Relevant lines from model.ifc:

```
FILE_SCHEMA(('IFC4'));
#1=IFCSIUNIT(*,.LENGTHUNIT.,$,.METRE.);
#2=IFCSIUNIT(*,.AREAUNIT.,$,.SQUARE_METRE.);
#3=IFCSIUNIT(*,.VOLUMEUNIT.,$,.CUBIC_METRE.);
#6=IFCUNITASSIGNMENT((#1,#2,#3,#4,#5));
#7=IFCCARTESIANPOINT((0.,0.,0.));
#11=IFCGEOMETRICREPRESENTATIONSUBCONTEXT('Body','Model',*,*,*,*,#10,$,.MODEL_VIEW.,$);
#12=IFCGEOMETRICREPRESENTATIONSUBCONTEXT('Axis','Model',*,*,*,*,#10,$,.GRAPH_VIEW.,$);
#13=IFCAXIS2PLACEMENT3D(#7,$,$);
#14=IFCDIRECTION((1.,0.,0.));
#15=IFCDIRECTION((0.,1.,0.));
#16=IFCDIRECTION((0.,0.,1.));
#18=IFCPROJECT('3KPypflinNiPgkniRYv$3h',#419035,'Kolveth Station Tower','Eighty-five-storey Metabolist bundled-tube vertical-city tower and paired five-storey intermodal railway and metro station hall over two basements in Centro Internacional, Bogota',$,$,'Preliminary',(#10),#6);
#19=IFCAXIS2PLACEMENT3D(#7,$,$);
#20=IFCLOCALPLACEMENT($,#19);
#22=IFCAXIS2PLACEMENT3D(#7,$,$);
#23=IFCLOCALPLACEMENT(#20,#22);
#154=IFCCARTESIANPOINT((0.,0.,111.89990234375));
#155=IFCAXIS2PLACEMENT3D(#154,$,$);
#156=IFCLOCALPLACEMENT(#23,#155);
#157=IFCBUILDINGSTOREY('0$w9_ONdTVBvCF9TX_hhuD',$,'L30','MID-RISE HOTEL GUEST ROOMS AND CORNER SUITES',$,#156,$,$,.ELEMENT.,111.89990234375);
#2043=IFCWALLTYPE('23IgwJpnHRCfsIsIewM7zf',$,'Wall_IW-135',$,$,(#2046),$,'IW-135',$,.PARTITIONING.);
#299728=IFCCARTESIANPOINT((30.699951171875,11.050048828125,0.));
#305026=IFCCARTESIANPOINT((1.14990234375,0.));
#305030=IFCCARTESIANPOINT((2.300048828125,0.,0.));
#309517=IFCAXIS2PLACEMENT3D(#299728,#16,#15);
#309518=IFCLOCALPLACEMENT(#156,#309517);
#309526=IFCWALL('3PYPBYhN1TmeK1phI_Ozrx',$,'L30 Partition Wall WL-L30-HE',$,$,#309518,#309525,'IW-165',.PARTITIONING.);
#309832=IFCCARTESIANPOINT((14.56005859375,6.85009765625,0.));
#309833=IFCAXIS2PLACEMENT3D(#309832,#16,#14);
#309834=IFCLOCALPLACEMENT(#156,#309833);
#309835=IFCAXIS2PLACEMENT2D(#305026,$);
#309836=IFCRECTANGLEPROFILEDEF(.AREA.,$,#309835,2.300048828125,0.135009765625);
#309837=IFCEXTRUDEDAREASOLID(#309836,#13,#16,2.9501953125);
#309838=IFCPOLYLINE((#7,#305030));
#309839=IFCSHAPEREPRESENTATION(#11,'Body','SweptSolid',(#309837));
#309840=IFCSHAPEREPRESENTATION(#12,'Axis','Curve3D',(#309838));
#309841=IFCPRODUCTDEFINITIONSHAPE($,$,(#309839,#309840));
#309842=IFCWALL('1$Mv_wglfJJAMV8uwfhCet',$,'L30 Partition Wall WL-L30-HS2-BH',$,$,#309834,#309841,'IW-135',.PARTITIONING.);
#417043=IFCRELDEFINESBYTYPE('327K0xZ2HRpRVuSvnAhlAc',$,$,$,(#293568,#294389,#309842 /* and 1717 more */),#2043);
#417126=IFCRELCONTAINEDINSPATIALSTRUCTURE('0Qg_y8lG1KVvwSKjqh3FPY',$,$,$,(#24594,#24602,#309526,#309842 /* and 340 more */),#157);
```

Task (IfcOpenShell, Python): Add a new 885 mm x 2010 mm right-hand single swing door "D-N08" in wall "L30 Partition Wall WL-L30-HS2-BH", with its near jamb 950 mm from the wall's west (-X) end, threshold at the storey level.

```python
import numpy as np
import ifcopenshell
import ifcopenshell.api.feature
import ifcopenshell.api.geometry
import ifcopenshell.api.root
import ifcopenshell.api.spatial
import ifcopenshell.geom
import ifcopenshell.util.element
import ifcopenshell.util.placement
import ifcopenshell.util.representation
import ifcopenshell.util.shape
import ifcopenshell.util.unit

model = ifcopenshell.open("model.ifc")
unit_scale = ifcopenshell.util.unit.calculate_unit_scale(model)
settings = ifcopenshell.geom.settings()


def volume(element):
    """Net volume in cubic metres, openings subtracted."""
    shape = ifcopenshell.geom.create_shape(settings, element)
    return ifcopenshell.util.shape.get_volume(shape.geometry)


wall = model.by_guid("1$Mv_wglfJJAMV8uwfhCet")
storey = ifcopenshell.util.element.get_container(wall, ifc_class="IfcBuildingStorey")
context = ifcopenshell.util.representation.get_context(model, "Model", "Body", "MODEL_VIEW")
before = volume(wall)

width, height, from_end, sill = 0.885, 2.01, 0.95, 0.0  # metres

# The wall runs along its own X axis, and the end named is its -X end.
wall_shape = ifcopenshell.geom.create_shape(settings, wall)
x, y, z = ifcopenshell.util.shape.get_vertices(wall_shape.geometry).T
start = x.min() + from_end
face, thickness = float(y.min()), float(y.max() - y.min())
wall_matrix = ifcopenshell.util.placement.get_local_placement(wall.ObjectPlacement)
level = ifcopenshell.util.placement.get_local_placement(storey.ObjectPlacement)[2, 3]


def in_wall(x, y):
    """Placement at x, y metres in the wall's axes, at sill height."""
    matrix = wall_matrix.copy()
    matrix[:, 3] = wall_matrix @ np.array([x / unit_scale, y / unit_scale, 0.0, 1.0])
    matrix[2, 3] = level + sill / unit_scale
    return matrix


# Opening: a box that overshoots both wall faces by 50 mm.
opening = ifcopenshell.api.root.create_entity(model, ifc_class="IfcOpeningElement", predefined_type="OPENING")
box = ifcopenshell.api.geometry.add_wall_representation(
    model, context=context, length=width, height=height, thickness=thickness + 0.1
)
ifcopenshell.api.geometry.assign_representation(model, product=opening, representation=box)
ifcopenshell.api.geometry.edit_object_placement(model, product=opening, matrix=in_wall(start, face - 0.05), is_si=False)
ifcopenshell.api.feature.add_feature(model, feature=opening, element=wall)

door = ifcopenshell.api.root.create_entity(model, ifc_class="IfcDoor", name="D-N08", predefined_type="DOOR")
door.OverallWidth, door.OverallHeight = width / unit_scale, height / unit_scale
door.OperationType = "SINGLE_SWING_RIGHT"
body = ifcopenshell.api.geometry.add_door_representation(
    model,
    context=context,
    overall_width=door.OverallWidth,
    overall_height=door.OverallHeight,
    operation_type="SINGLE_SWING_RIGHT",
    lining_properties={"LiningDepth": thickness / unit_scale, "ThresholdDepth": thickness / unit_scale},
)
ifcopenshell.api.geometry.assign_representation(model, product=door, representation=body)
ifcopenshell.api.spatial.assign_container(model, products=[door], relating_structure=storey)
ifcopenshell.api.feature.add_filling(model, opening=opening, element=door)

# The lining spans the wall, so the door starts at the wall face.
ifcopenshell.api.geometry.edit_object_placement(model, product=door, matrix=in_wall(start, face), is_si=False)

after = volume(wall)

print(f"wall volume {before:.3f} -> {after:.3f} m3")

model.write("model_rev.ifc")
```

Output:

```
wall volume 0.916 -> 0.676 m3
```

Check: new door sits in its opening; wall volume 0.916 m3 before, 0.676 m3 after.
